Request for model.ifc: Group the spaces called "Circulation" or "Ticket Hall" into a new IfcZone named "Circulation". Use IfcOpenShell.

First a look at what the model holds.

```python
import ifcopenshell

model = ifcopenshell.open("model.ifc")
print(model.schema)
seen = {}
for space in model.by_type("IfcSpace"):
    seen[space.LongName] = seen.get(space.LongName, 0) + 1
for name, count in sorted(seen.items(), key=str):
    print(count, "x", name)
print("zones:", [z.Name for z in model.by_type("IfcZone")][:20])
```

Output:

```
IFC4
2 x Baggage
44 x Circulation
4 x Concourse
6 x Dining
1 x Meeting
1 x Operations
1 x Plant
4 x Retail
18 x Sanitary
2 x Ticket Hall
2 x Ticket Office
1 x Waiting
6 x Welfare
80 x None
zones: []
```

```python
import ifcopenshell
import ifcopenshell.api.group
import ifcopenshell.api.root

model = ifcopenshell.open("model.ifc")

names = {"Circulation", "Ticket Hall"}
spaces = [s for s in model.by_type("IfcSpace") if s.LongName in names]

zone = ifcopenshell.api.root.create_entity(model, ifc_class="IfcZone", name="Circulation")
ifcopenshell.api.group.assign_group(model, products=spaces, group=zone)
print(len(spaces), "spaces in", zone.Name)

model.write("model_rev.ifc")
```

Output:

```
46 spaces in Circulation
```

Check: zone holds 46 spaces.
